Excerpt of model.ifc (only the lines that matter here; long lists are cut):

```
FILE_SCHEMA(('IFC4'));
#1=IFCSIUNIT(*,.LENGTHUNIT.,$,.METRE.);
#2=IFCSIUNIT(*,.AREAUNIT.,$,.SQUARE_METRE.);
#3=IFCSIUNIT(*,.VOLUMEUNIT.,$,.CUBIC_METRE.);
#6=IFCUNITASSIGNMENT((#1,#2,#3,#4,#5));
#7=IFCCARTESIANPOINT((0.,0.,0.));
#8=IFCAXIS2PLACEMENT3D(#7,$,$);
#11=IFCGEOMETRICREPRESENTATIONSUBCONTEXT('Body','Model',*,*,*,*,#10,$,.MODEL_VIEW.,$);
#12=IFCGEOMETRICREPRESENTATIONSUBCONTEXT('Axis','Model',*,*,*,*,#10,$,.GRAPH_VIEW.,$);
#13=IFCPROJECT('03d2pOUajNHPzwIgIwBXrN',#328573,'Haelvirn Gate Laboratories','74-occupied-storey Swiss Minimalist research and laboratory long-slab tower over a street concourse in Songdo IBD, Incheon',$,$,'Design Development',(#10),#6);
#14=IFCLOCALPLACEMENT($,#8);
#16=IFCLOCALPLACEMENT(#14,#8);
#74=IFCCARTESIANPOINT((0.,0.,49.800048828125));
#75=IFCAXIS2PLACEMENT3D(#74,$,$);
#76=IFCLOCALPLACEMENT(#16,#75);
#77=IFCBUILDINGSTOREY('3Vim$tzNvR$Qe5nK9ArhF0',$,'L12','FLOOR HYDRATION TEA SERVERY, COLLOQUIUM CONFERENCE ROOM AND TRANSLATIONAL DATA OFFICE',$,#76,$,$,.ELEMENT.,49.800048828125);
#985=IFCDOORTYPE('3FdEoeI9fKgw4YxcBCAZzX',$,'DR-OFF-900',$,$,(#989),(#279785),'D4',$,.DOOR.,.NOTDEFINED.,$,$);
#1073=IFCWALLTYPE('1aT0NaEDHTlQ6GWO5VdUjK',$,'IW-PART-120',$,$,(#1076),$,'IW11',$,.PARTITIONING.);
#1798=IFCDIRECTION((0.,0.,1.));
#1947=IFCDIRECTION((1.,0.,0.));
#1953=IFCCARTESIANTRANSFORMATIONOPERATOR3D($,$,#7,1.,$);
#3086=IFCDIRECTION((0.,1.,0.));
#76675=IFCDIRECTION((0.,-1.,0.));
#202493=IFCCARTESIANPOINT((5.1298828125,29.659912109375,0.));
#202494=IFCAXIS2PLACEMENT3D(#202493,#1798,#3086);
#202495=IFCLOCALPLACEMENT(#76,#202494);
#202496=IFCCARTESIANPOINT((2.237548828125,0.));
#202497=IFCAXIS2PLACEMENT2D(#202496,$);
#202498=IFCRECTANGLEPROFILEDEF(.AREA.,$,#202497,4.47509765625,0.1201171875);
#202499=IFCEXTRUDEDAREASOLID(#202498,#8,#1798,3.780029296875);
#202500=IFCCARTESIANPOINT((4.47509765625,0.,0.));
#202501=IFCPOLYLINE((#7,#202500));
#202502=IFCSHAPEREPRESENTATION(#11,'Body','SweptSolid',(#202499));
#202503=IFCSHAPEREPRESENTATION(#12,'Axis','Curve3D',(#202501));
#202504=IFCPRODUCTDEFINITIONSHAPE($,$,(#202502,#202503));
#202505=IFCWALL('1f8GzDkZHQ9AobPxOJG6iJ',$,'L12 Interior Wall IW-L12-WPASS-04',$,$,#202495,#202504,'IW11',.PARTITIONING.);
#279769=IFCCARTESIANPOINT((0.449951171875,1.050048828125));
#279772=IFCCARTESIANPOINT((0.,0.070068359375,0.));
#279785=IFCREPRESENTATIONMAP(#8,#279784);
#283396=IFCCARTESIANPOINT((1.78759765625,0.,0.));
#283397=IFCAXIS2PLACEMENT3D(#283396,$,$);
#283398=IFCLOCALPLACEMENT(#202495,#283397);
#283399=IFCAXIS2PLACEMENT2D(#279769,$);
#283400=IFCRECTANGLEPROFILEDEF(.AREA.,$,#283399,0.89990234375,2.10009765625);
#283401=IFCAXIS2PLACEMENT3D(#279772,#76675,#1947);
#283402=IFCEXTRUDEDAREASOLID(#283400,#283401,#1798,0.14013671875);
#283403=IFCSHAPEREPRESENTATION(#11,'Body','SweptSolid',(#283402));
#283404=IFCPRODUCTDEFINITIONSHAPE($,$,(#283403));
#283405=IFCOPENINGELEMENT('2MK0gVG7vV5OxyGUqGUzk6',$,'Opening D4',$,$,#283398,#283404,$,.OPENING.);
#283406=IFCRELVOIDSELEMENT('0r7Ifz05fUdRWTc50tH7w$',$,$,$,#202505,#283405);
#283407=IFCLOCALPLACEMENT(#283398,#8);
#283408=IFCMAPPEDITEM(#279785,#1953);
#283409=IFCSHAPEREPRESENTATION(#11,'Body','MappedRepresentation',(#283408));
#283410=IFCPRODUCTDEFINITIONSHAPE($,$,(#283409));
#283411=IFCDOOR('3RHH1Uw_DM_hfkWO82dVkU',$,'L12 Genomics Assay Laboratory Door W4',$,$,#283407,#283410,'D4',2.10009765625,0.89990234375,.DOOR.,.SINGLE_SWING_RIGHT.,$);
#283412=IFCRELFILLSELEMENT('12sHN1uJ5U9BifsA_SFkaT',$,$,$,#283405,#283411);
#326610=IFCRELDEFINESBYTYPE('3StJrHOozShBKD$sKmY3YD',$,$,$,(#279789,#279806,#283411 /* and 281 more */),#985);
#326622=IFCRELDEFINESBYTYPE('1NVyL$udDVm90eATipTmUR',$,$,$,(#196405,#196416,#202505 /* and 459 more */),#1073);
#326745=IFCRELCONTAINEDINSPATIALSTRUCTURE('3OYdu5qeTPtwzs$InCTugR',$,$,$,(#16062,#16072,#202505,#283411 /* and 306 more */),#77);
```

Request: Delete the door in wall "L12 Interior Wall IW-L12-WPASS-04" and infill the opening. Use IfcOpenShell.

```python
import ifcopenshell
import ifcopenshell.api.feature
import ifcopenshell.api.root
import ifcopenshell.geom
import ifcopenshell.util.shape

model = ifcopenshell.open("model.ifc")
settings = ifcopenshell.geom.settings()


def volume(element):
    """Net volume in cubic metres, openings subtracted."""
    shape = ifcopenshell.geom.create_shape(settings, element)
    return ifcopenshell.util.shape.get_volume(shape.geometry)


door = model.by_id(283411)
opening = door.FillsVoids[0].RelatingOpeningElement
wall = opening.VoidsElements[0].RelatingBuildingElement
before = volume(wall)

ifcopenshell.api.root.remove_product(model, product=door)
ifcopenshell.api.feature.remove_feature(model, feature=opening)

after = volume(wall)

print(f"wall volume {before:.3f} -> {after:.3f} m3")

model.write("model-out.ifc")
```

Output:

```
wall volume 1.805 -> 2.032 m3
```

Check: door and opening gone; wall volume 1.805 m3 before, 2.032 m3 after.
